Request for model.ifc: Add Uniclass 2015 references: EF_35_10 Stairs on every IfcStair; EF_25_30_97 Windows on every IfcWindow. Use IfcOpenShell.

First a look at what the model holds.

```python
import ifcopenshell

model = ifcopenshell.open("model.ifc")
print(model.schema)
print("classifications:", [c.Name for c in model.by_type("IfcClassification")])
for ifc_class in ("IfcDoor", "IfcRoof", "IfcStair", "IfcWall", "IfcWindow"):
    print(ifc_class, len(model.by_type(ifc_class)))
```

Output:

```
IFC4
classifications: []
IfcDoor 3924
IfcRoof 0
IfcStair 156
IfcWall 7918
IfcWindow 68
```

```python
import ifcopenshell
import ifcopenshell.api.classification

model = ifcopenshell.open("model.ifc")

system = ifcopenshell.api.classification.add_classification(model, classification="Uniclass 2015")

codes = {
    "IfcStair": ("EF_35_10", "Stairs"),
    "IfcWindow": ("EF_25_30_97", "Windows"),
}
for ifc_class, (code, name) in codes.items():
    products = model.by_type(ifc_class)
    ifcopenshell.api.classification.add_reference(
        model, products=products, classification=system, identification=code, name=name
    )
    print(code, len(products))

model.write("model_edited.ifc")
```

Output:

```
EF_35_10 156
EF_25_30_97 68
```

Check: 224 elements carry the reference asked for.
